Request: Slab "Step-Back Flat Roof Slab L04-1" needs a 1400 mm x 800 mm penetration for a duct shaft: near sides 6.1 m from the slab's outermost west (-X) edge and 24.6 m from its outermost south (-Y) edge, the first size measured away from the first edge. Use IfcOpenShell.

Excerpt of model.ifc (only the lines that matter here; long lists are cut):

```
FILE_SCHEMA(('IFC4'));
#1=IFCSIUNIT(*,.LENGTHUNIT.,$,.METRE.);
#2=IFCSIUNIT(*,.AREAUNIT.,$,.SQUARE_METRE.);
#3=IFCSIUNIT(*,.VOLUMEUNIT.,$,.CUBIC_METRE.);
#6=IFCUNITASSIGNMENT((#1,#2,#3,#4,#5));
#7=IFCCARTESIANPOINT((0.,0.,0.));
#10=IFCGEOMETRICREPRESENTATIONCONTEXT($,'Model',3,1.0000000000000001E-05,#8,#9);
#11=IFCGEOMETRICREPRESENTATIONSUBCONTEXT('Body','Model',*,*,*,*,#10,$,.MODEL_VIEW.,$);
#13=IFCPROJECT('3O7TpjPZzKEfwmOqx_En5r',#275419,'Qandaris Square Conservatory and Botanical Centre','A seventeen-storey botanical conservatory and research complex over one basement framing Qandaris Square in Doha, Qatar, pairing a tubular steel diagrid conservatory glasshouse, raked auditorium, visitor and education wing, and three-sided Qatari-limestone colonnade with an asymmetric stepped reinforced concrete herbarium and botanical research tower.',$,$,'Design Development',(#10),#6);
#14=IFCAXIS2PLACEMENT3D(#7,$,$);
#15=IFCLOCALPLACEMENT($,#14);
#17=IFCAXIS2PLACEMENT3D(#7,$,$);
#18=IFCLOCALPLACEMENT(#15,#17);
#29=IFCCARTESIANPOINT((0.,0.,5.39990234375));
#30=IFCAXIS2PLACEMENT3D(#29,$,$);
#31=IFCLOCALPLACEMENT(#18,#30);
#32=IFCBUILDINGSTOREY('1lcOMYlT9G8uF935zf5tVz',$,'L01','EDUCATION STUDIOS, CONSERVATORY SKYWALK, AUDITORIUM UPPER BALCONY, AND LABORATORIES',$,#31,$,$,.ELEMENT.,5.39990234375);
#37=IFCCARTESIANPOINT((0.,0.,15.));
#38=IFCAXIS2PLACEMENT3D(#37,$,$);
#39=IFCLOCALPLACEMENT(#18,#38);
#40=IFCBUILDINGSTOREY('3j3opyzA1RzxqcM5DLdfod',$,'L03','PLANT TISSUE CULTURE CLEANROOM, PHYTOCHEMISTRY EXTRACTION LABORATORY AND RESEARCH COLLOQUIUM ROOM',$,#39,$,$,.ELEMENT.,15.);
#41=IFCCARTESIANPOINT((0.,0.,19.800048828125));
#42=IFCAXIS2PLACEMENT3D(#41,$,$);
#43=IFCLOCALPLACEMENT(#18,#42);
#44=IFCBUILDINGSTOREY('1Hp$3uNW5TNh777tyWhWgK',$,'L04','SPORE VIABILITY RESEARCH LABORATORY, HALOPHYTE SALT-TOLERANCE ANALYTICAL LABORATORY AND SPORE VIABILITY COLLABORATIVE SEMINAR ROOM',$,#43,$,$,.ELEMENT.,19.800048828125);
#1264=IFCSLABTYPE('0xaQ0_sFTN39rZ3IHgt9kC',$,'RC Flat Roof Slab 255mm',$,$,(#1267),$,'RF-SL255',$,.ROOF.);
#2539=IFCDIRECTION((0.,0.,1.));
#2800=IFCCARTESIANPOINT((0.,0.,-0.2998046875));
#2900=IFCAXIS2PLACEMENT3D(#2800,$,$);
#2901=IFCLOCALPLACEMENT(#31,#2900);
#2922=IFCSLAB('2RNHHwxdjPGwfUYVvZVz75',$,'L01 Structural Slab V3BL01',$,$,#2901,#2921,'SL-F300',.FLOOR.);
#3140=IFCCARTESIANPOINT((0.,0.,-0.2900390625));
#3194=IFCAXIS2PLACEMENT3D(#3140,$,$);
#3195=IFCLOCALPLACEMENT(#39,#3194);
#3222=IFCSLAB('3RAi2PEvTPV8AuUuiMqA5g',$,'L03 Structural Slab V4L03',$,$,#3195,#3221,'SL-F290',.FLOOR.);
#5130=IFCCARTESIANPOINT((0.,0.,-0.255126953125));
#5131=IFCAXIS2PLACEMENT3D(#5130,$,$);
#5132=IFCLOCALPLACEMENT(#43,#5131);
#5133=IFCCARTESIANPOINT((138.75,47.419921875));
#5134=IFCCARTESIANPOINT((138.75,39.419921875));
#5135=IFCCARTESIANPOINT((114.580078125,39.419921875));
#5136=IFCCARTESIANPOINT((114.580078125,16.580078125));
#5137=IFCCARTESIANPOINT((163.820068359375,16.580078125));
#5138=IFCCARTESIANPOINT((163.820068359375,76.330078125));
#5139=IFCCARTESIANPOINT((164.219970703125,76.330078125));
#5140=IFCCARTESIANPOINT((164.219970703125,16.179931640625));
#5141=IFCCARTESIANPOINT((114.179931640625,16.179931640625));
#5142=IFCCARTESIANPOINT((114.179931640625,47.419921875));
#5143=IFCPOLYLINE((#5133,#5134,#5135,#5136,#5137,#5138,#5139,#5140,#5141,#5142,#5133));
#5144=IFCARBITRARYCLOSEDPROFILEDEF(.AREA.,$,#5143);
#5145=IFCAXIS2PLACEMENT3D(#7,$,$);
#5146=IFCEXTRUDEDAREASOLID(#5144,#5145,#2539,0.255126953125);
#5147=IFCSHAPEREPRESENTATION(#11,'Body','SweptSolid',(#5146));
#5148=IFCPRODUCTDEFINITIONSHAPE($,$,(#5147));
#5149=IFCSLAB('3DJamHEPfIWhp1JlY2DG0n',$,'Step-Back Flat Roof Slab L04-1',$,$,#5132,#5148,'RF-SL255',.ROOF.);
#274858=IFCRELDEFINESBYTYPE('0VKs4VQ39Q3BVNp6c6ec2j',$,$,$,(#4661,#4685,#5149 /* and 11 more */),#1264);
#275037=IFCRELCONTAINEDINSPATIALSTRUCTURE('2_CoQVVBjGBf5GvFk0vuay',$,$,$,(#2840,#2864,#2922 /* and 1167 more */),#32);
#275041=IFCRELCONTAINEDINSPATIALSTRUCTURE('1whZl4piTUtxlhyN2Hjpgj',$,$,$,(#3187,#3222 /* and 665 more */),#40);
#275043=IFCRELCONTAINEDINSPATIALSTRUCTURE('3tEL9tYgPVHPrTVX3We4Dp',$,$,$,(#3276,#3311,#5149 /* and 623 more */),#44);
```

```python
import numpy as np
import ifcopenshell
import ifcopenshell.api.feature
import ifcopenshell.api.geometry
import ifcopenshell.api.root
import ifcopenshell.geom
import ifcopenshell.util.placement
import ifcopenshell.util.representation
import ifcopenshell.util.shape
import ifcopenshell.util.unit

model = ifcopenshell.open("model.ifc")
unit_scale = ifcopenshell.util.unit.calculate_unit_scale(model)
settings = ifcopenshell.geom.settings()


def volume(element):
    """Net volume in cubic metres, openings subtracted."""
    shape = ifcopenshell.geom.create_shape(settings, element)
    return ifcopenshell.util.shape.get_volume(shape.geometry)


slab = model.by_guid("3DJamHEPfIWhp1JlY2DG0n")
before = volume(slab)

# Extent in the slab's own axes, in metres. The edges named are its -X and -Y sides.
slab_shape = ifcopenshell.geom.create_shape(settings, slab)
vertices = ifcopenshell.util.shape.get_vertices(slab_shape.geometry)
x_min, y_min, bottom = vertices.min(axis=0)
top = vertices[:, 2].max()

opening = ifcopenshell.api.root.create_entity(model, ifc_class="IfcOpeningElement", name="Duct shaft opening", predefined_type="OPENING")
context = ifcopenshell.util.representation.get_context(model, "Model", "Body", "MODEL_VIEW")
width, depth = 1.4, 0.8
outline = [(0.0, 0.0), (width, 0.0), (width, depth), (0.0, depth), (0.0, 0.0)]
# Overshoot both faces by 50 mm so the cut is clean.
shape = ifcopenshell.api.geometry.add_slab_representation(
    model, context=context, depth=top - bottom + 0.1, polyline=outline
)
ifcopenshell.api.geometry.assign_representation(model, product=opening, representation=shape)

matrix = ifcopenshell.util.placement.get_local_placement(slab.ObjectPlacement)
matrix[:, 3] = matrix @ np.append(np.array([x_min + 6.1, y_min + 24.6, bottom - 0.05]) / unit_scale, 1.0)
ifcopenshell.api.geometry.edit_object_placement(model, product=opening, matrix=matrix, is_si=False)
ifcopenshell.api.feature.add_feature(model, feature=opening, element=slab)

after = volume(slab)

print(f"slab volume {before:.3f} -> {after:.3f} m3")

model.write("model_updated.ifc")
```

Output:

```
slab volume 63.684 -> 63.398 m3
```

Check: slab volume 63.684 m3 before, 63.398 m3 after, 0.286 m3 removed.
